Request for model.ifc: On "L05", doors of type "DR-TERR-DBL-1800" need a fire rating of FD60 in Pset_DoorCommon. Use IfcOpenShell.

First a look at what the model holds.

```python
import ifcopenshell
import ifcopenshell.util.element

model = ifcopenshell.open("model.ifc")
print(model.schema)
storey = next(s for s in model.by_type("IfcBuildingStorey") if s.Name == "L05")
doors = [e for e in ifcopenshell.util.element.get_decomposition(storey) if e.is_a("IfcDoor")]
seen = {}
for e in doors:
    element_type = ifcopenshell.util.element.get_type(e)
    key = (element_type.Name if element_type != e and element_type else None, ifcopenshell.util.element.get_pset(e, "Pset_DoorCommon", "FireRating"))
    seen[key] = seen.get(key, 0) + 1
for (name, value), count in sorted(seen.items(), key=str):
    print(count, "x", name, "|", value)
```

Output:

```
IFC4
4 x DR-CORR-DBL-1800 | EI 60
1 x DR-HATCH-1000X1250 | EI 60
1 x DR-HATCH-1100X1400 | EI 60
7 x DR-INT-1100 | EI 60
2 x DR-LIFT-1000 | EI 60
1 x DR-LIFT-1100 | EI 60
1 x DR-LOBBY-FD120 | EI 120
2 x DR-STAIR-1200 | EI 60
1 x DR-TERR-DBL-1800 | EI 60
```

```python
import ifcopenshell
import ifcopenshell.api.pset
import ifcopenshell.util.element

model = ifcopenshell.open("model.ifc")

storey = next(s for s in model.by_type("IfcBuildingStorey") if s.Name == "L05")
doors = [e for e in ifcopenshell.util.element.get_decomposition(storey) if e.is_a("IfcDoor")]

count = 0
for e in doors:
    element_type = ifcopenshell.util.element.get_type(e)
    if element_type in (None, e) or element_type.Name != "DR-TERR-DBL-1800":
        continue
    # add_pset returns the element's existing set when there is one.
    pset = ifcopenshell.api.pset.add_pset(model, product=e, name="Pset_DoorCommon")
    ifcopenshell.api.pset.edit_pset(model, pset=pset, properties={"FireRating": "FD60"})
    count += 1

print(count, "doors updated")

model.write("model_edited.ifc")
```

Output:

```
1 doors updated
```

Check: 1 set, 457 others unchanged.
